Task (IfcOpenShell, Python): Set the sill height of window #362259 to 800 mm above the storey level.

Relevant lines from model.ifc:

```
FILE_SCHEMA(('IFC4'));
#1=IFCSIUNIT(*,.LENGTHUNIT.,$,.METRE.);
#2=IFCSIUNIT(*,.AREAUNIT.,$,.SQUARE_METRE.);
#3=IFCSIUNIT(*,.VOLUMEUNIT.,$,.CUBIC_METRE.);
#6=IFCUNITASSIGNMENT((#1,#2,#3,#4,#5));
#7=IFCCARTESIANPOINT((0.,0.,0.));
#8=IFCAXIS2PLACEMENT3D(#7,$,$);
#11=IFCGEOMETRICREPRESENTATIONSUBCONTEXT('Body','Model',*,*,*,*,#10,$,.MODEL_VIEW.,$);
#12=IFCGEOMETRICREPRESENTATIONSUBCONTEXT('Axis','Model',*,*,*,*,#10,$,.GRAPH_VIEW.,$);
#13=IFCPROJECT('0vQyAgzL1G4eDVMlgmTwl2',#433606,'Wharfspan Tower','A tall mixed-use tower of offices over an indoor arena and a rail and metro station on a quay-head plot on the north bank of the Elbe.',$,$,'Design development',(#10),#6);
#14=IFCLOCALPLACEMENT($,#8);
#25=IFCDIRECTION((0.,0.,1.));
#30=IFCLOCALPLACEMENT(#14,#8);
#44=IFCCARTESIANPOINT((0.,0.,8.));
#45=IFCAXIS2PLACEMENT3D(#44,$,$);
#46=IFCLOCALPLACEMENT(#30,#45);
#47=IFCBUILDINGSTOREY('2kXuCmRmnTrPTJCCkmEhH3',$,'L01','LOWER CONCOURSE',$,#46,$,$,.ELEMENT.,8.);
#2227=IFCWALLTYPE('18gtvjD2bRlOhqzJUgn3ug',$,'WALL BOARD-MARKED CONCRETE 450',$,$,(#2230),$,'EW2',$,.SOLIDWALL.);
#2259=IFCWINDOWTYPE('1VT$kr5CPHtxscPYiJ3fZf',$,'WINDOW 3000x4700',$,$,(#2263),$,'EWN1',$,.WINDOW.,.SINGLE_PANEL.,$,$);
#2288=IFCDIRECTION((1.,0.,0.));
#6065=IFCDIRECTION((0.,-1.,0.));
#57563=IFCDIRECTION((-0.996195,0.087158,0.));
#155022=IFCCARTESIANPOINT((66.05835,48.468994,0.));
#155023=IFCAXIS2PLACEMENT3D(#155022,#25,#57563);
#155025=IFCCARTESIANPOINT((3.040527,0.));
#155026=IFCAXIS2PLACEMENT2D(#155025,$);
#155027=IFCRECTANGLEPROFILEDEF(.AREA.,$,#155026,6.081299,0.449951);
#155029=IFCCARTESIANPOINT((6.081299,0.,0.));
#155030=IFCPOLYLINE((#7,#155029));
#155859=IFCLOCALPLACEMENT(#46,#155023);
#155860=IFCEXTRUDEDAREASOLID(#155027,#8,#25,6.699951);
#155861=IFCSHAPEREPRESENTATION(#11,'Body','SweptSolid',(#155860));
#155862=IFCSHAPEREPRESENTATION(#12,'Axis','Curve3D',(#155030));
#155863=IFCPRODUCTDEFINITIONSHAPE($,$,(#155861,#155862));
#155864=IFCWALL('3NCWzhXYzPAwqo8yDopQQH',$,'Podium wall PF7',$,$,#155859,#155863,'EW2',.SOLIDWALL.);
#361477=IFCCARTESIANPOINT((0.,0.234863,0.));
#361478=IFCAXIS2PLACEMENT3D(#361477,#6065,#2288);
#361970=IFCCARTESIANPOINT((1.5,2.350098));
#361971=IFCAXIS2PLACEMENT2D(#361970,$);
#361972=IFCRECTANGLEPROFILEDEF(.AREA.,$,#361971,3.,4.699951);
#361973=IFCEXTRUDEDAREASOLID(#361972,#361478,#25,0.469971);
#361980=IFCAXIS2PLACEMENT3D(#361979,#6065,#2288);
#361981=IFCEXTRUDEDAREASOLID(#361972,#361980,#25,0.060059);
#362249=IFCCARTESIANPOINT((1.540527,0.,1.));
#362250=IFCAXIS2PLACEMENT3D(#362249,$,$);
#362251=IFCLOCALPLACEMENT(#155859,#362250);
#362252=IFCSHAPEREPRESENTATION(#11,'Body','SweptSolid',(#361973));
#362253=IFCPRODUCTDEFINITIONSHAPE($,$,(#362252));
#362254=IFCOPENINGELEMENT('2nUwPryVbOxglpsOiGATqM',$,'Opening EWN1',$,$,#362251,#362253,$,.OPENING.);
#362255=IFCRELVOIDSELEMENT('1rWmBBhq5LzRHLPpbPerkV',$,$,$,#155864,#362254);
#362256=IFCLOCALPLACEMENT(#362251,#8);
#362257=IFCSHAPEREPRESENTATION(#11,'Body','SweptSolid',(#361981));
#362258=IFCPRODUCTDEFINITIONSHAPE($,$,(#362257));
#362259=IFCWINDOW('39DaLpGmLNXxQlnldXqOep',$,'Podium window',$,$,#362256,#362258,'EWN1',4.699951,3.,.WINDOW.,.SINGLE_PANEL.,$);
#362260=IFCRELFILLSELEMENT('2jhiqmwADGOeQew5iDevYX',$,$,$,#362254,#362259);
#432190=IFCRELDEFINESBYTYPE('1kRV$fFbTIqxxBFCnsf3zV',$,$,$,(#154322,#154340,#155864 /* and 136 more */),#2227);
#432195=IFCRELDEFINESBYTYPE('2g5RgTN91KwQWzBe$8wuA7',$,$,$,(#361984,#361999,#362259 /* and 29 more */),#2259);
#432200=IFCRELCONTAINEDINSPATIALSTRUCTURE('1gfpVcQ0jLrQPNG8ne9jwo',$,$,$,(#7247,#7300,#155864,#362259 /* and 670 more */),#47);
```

```python
import numpy as np
import ifcopenshell
import ifcopenshell.api.geometry
import ifcopenshell.geom
import ifcopenshell.util.element
import ifcopenshell.util.placement
import ifcopenshell.util.shape
import ifcopenshell.util.unit

model = ifcopenshell.open("model.ifc")
unit_scale = ifcopenshell.util.unit.calculate_unit_scale(model)

window = model.by_id(362259)
opening = window.FillsVoids[0].RelatingOpeningElement
storey = ifcopenshell.util.element.get_container(window, ifc_class="IfcBuildingStorey")
level = ifcopenshell.util.placement.get_local_placement(storey.ObjectPlacement)[2, 3]

# The opening's origin need not be at the sill, so measure its lowest point.
shape = ifcopenshell.geom.create_shape(ifcopenshell.geom.settings(), opening)
bottom = ifcopenshell.util.shape.get_shape_bottom_elevation(shape, shape.geometry) / unit_scale
dz = level + 0.8 / unit_scale - bottom

shift = np.array([0.0, 0.0, dz])
# The window is placed relative to its opening, so it follows when the opening moves.
matrix = ifcopenshell.util.placement.get_local_placement(opening.ObjectPlacement)
matrix[:3, 3] += shift
ifcopenshell.api.geometry.edit_object_placement(
    model, product=opening, matrix=matrix, is_si=False, should_transform_children=True
)

print(f"moved by {dz * unit_scale:+.3f} m")

model.write("model_updated.ifc")
```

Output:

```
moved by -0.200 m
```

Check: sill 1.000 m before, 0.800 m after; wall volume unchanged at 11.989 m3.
